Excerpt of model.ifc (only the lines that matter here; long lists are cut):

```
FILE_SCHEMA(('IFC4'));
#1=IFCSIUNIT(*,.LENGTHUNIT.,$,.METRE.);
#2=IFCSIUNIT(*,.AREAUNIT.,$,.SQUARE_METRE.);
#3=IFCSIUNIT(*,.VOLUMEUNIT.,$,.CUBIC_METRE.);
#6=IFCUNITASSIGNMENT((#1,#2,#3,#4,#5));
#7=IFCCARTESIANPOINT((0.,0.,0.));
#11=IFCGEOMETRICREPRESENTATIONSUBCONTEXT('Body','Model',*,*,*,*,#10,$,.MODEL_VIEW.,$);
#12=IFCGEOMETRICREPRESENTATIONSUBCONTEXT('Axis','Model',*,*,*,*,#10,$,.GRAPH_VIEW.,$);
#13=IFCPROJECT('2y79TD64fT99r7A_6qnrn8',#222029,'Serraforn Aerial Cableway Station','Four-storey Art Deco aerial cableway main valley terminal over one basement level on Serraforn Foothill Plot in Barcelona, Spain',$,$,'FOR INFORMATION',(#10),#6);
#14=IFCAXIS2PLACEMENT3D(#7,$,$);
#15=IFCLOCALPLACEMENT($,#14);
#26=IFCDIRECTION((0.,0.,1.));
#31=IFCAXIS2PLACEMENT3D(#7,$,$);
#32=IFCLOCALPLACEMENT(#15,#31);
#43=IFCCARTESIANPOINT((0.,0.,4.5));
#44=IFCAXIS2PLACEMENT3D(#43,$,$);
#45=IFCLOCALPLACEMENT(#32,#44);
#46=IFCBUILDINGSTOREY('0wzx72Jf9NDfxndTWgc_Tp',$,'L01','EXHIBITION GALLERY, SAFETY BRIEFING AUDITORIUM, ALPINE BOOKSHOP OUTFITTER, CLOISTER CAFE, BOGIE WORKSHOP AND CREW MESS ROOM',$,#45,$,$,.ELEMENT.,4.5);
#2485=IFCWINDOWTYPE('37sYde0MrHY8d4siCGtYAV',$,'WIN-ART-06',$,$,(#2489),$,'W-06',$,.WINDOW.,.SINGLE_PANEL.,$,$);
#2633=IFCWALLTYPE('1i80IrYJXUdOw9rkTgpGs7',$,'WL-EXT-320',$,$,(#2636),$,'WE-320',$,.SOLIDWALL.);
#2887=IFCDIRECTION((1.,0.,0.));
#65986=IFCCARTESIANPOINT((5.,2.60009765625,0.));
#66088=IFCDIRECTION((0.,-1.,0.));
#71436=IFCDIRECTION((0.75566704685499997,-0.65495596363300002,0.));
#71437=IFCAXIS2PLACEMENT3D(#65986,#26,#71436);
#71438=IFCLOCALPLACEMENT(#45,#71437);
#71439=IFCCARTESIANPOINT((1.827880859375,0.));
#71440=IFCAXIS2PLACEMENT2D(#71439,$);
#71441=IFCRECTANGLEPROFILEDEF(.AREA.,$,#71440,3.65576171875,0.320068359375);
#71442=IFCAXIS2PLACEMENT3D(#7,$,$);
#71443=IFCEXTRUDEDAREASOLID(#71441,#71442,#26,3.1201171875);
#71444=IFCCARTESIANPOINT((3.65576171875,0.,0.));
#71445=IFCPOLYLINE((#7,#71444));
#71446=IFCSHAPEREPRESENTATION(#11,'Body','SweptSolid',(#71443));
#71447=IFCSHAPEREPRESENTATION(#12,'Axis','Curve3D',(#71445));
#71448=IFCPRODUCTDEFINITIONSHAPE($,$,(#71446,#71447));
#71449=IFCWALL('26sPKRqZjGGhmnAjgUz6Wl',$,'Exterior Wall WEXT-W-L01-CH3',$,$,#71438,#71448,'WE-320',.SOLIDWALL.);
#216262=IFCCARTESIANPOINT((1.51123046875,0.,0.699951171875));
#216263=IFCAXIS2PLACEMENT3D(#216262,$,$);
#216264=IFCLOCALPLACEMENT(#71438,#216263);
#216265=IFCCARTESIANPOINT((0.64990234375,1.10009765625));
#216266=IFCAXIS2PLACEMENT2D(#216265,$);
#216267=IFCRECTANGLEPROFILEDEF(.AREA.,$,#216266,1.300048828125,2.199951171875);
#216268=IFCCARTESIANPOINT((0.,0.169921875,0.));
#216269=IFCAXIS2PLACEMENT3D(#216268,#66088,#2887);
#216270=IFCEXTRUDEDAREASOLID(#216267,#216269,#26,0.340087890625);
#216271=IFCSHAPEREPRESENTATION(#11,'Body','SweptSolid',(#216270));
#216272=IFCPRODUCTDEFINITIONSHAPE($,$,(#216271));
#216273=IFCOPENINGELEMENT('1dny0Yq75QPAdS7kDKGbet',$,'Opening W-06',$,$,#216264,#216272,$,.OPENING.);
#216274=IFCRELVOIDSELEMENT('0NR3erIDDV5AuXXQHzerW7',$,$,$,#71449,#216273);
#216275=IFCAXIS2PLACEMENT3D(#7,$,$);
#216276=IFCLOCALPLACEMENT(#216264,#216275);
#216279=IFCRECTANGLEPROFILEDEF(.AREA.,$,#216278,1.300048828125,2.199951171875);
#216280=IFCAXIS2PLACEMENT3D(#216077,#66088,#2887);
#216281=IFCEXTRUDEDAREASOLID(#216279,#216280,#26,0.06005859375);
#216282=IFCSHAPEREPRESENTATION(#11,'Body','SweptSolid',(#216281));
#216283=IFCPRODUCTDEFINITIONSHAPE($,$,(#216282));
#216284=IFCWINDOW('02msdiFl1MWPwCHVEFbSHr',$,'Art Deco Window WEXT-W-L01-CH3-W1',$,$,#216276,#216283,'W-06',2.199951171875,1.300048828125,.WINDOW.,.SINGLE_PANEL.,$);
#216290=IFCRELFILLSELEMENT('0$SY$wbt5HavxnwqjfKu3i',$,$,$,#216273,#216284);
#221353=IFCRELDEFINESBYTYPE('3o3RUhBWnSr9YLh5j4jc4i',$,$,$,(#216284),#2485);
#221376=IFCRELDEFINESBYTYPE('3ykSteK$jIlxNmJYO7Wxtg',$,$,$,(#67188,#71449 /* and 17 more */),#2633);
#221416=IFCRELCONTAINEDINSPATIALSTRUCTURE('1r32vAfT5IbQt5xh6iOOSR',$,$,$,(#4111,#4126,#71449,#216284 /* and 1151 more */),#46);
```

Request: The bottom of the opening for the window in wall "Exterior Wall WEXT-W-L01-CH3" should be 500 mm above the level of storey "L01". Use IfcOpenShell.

```python
import numpy as np
import ifcopenshell
import ifcopenshell.api.geometry
import ifcopenshell.geom
import ifcopenshell.util.element
import ifcopenshell.util.placement
import ifcopenshell.util.shape
import ifcopenshell.util.unit

model = ifcopenshell.open("model.ifc")
unit_scale = ifcopenshell.util.unit.calculate_unit_scale(model)

window = model.by_guid("02msdiFl1MWPwCHVEFbSHr")
opening = window.FillsVoids[0].RelatingOpeningElement
storey = ifcopenshell.util.element.get_container(window, ifc_class="IfcBuildingStorey")
level = ifcopenshell.util.placement.get_local_placement(storey.ObjectPlacement)[2, 3]

# The opening's origin need not be at the sill, so measure its lowest point.
shape = ifcopenshell.geom.create_shape(ifcopenshell.geom.settings(), opening)
bottom = ifcopenshell.util.shape.get_shape_bottom_elevation(shape, shape.geometry) / unit_scale
dz = level + 0.5 - bottom

shift = np.array([0.0, 0.0, dz])
# The window is placed relative to its opening, so it follows when the opening moves.
matrix = ifcopenshell.util.placement.get_local_placement(opening.ObjectPlacement)
matrix[:3, 3] += shift
ifcopenshell.api.geometry.edit_object_placement(
    model, product=opening, matrix=matrix, is_si=False, should_transform_children=True
)

print(f"moved by {dz * unit_scale:+.3f} m")

model.write("model_v2.ifc")
```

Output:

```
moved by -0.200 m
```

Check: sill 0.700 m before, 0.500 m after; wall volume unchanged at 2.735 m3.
